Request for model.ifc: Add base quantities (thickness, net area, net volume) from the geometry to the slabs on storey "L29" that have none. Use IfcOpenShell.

First a look at what the model holds.

```python
import ifcopenshell
import ifcopenshell.util.element
import ifcopenshell.util.unit

model = ifcopenshell.open("model.ifc")
print(model.schema)
for unit_type in ("LENGTHUNIT", "AREAUNIT", "VOLUMEUNIT"):
    print(unit_type, ifcopenshell.util.unit.calculate_unit_scale(model, unit_type))
storey = next(s for s in model.by_type("IfcBuildingStorey") if s.Name == "L29")
slabs = [e for e in ifcopenshell.util.element.get_decomposition(storey) if e.is_a("IfcSlab")]
for e in sorted(slabs, key=lambda e: e.id()):
    print(e.id(), e.is_a(), e.Name, list(ifcopenshell.util.element.get_psets(e, qtos_only=True)), sep=" | ")
```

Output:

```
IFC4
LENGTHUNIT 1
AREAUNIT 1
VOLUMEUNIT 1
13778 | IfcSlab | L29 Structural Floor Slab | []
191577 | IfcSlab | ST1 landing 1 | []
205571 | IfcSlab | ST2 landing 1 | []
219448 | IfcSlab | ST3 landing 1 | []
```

```python
import ifcopenshell
import ifcopenshell.api.pset
import ifcopenshell.geom
import ifcopenshell.util.element
import ifcopenshell.util.shape
import ifcopenshell.util.unit

model = ifcopenshell.open("model.ifc")
unit_scale = ifcopenshell.util.unit.calculate_unit_scale(model)
area_scale = ifcopenshell.util.unit.calculate_unit_scale(model, "AREAUNIT")
volume_scale = ifcopenshell.util.unit.calculate_unit_scale(model, "VOLUMEUNIT")
settings = ifcopenshell.geom.settings()

storey = next(s for s in model.by_type("IfcBuildingStorey") if s.Name == "L29")
slabs = [e for e in ifcopenshell.util.element.get_decomposition(storey) if e.is_a("IfcSlab")]

for e in sorted(slabs, key=lambda e: e.id()):
    if ifcopenshell.util.element.get_psets(e, qtos_only=True, should_inherit=False):
        continue
    # Geometry comes back in metres, in the element's own axes.
    shape = ifcopenshell.geom.create_shape(settings, e)
    values = {
        "Width": ifcopenshell.util.shape.get_z(shape.geometry) / unit_scale,
        "NetArea": ifcopenshell.util.shape.get_footprint_area(shape.geometry) / area_scale,
        "NetVolume": ifcopenshell.util.shape.get_volume(shape.geometry) / volume_scale,
    }
    qto = ifcopenshell.api.pset.add_qto(model, product=e, name="Qto_SlabBaseQuantities")
    ifcopenshell.api.pset.edit_qto(model, qto=qto, properties=values)
    print(e.id(), {k: round(v, 3) for k, v in values.items()})

model.write("model_rev.ifc")
```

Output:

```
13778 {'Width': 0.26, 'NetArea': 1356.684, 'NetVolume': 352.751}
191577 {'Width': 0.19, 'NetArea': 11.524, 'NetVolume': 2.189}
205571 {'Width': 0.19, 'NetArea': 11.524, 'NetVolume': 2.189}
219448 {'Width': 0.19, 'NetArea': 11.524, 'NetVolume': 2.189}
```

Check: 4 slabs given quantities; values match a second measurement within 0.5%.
